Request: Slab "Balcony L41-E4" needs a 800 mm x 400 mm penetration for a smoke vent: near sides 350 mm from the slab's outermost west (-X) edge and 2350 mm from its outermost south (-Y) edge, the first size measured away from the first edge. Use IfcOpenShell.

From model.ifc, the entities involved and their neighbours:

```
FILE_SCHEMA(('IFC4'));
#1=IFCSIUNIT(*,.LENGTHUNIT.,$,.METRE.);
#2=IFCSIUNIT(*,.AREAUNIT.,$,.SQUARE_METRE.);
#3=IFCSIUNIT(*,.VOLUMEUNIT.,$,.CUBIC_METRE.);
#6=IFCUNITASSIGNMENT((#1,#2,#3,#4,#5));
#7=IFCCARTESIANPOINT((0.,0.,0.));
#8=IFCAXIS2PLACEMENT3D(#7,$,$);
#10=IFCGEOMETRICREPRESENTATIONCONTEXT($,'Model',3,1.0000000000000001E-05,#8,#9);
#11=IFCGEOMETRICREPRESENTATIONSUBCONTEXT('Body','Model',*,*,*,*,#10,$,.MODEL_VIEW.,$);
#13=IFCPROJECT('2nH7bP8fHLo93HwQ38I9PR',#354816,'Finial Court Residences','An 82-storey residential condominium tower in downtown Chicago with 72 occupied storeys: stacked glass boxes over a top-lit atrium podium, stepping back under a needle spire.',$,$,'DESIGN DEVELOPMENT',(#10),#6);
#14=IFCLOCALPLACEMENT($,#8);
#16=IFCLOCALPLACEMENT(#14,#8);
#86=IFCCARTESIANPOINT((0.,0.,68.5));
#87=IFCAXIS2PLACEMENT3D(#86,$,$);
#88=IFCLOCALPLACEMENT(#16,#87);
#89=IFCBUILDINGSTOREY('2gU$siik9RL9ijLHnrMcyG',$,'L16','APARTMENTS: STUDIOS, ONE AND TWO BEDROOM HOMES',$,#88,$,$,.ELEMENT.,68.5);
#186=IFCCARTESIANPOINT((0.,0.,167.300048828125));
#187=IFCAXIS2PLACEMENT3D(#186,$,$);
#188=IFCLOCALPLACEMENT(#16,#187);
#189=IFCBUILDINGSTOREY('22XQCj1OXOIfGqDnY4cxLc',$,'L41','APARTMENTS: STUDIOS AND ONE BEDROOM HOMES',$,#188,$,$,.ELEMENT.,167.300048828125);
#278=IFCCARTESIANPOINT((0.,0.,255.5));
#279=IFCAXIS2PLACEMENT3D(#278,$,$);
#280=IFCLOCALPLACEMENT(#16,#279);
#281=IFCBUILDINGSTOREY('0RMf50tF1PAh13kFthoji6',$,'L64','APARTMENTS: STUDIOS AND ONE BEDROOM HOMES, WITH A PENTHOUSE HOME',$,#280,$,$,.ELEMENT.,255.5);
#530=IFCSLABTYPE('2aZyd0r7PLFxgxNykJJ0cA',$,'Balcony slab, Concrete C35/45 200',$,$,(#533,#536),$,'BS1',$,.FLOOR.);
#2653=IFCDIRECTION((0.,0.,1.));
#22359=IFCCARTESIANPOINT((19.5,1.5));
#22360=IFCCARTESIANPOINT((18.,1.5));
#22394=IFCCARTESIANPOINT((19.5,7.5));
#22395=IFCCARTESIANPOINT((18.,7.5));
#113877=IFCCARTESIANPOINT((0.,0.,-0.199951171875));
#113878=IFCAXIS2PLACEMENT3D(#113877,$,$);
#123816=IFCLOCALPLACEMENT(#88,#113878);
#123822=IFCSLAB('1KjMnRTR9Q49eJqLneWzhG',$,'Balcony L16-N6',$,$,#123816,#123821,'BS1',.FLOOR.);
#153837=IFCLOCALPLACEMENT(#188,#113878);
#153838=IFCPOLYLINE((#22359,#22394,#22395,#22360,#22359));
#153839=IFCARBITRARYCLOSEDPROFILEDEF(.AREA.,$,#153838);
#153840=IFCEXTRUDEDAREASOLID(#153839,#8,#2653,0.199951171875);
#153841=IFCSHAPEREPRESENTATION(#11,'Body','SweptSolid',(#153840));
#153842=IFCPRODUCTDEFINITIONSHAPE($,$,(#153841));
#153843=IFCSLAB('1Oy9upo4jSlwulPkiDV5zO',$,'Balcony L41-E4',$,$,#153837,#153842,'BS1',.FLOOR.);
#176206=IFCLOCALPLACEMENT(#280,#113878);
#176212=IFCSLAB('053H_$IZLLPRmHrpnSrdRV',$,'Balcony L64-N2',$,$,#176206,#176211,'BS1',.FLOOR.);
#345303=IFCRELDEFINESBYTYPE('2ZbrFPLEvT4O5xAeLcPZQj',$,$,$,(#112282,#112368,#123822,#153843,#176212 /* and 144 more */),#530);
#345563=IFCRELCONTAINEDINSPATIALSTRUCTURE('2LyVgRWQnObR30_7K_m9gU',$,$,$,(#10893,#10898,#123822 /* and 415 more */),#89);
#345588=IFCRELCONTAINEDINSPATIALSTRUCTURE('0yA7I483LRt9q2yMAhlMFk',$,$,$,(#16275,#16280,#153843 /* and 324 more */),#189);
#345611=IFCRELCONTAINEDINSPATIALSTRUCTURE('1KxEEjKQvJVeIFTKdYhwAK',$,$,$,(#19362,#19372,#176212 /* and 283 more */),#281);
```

```python
import numpy as np
import ifcopenshell
import ifcopenshell.api.feature
import ifcopenshell.api.geometry
import ifcopenshell.api.root
import ifcopenshell.geom
import ifcopenshell.util.placement
import ifcopenshell.util.representation
import ifcopenshell.util.shape
import ifcopenshell.util.unit

model = ifcopenshell.open("model.ifc")
unit_scale = ifcopenshell.util.unit.calculate_unit_scale(model)
settings = ifcopenshell.geom.settings()


def volume(element):
    """Net volume in cubic metres, openings subtracted."""
    shape = ifcopenshell.geom.create_shape(settings, element)
    return ifcopenshell.util.shape.get_volume(shape.geometry)


slab = model.by_id(153843)
before = volume(slab)

# Extent in the slab's own axes, in metres. The edges named are its -X and -Y sides.
slab_shape = ifcopenshell.geom.create_shape(settings, slab)
vertices = ifcopenshell.util.shape.get_vertices(slab_shape.geometry)
x_min, y_min, bottom = vertices.min(axis=0)
top = vertices[:, 2].max()

opening = ifcopenshell.api.root.create_entity(model, ifc_class="IfcOpeningElement", name="Smoke vent opening", predefined_type="OPENING")
context = ifcopenshell.util.representation.get_context(model, "Model", "Body", "MODEL_VIEW")
width, depth = 0.8, 0.4
outline = [(0.0, 0.0), (width, 0.0), (width, depth), (0.0, depth), (0.0, 0.0)]
# Overshoot both faces by 50 mm so the cut is clean.
shape = ifcopenshell.api.geometry.add_slab_representation(
    model, context=context, depth=top - bottom + 0.1, polyline=outline
)
ifcopenshell.api.geometry.assign_representation(model, product=opening, representation=shape)

matrix = ifcopenshell.util.placement.get_local_placement(slab.ObjectPlacement)
matrix[:, 3] = matrix @ np.append(np.array([x_min + 0.35, y_min + 2.35, bottom - 0.05]) / unit_scale, 1.0)
ifcopenshell.api.geometry.edit_object_placement(model, product=opening, matrix=matrix, is_si=False)
ifcopenshell.api.feature.add_feature(model, feature=opening, element=slab)

after = volume(slab)

print(f"slab volume {before:.3f} -> {after:.3f} m3")

model.write("model_edited.ifc")
```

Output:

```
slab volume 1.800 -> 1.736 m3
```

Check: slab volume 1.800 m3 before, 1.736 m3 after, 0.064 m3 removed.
